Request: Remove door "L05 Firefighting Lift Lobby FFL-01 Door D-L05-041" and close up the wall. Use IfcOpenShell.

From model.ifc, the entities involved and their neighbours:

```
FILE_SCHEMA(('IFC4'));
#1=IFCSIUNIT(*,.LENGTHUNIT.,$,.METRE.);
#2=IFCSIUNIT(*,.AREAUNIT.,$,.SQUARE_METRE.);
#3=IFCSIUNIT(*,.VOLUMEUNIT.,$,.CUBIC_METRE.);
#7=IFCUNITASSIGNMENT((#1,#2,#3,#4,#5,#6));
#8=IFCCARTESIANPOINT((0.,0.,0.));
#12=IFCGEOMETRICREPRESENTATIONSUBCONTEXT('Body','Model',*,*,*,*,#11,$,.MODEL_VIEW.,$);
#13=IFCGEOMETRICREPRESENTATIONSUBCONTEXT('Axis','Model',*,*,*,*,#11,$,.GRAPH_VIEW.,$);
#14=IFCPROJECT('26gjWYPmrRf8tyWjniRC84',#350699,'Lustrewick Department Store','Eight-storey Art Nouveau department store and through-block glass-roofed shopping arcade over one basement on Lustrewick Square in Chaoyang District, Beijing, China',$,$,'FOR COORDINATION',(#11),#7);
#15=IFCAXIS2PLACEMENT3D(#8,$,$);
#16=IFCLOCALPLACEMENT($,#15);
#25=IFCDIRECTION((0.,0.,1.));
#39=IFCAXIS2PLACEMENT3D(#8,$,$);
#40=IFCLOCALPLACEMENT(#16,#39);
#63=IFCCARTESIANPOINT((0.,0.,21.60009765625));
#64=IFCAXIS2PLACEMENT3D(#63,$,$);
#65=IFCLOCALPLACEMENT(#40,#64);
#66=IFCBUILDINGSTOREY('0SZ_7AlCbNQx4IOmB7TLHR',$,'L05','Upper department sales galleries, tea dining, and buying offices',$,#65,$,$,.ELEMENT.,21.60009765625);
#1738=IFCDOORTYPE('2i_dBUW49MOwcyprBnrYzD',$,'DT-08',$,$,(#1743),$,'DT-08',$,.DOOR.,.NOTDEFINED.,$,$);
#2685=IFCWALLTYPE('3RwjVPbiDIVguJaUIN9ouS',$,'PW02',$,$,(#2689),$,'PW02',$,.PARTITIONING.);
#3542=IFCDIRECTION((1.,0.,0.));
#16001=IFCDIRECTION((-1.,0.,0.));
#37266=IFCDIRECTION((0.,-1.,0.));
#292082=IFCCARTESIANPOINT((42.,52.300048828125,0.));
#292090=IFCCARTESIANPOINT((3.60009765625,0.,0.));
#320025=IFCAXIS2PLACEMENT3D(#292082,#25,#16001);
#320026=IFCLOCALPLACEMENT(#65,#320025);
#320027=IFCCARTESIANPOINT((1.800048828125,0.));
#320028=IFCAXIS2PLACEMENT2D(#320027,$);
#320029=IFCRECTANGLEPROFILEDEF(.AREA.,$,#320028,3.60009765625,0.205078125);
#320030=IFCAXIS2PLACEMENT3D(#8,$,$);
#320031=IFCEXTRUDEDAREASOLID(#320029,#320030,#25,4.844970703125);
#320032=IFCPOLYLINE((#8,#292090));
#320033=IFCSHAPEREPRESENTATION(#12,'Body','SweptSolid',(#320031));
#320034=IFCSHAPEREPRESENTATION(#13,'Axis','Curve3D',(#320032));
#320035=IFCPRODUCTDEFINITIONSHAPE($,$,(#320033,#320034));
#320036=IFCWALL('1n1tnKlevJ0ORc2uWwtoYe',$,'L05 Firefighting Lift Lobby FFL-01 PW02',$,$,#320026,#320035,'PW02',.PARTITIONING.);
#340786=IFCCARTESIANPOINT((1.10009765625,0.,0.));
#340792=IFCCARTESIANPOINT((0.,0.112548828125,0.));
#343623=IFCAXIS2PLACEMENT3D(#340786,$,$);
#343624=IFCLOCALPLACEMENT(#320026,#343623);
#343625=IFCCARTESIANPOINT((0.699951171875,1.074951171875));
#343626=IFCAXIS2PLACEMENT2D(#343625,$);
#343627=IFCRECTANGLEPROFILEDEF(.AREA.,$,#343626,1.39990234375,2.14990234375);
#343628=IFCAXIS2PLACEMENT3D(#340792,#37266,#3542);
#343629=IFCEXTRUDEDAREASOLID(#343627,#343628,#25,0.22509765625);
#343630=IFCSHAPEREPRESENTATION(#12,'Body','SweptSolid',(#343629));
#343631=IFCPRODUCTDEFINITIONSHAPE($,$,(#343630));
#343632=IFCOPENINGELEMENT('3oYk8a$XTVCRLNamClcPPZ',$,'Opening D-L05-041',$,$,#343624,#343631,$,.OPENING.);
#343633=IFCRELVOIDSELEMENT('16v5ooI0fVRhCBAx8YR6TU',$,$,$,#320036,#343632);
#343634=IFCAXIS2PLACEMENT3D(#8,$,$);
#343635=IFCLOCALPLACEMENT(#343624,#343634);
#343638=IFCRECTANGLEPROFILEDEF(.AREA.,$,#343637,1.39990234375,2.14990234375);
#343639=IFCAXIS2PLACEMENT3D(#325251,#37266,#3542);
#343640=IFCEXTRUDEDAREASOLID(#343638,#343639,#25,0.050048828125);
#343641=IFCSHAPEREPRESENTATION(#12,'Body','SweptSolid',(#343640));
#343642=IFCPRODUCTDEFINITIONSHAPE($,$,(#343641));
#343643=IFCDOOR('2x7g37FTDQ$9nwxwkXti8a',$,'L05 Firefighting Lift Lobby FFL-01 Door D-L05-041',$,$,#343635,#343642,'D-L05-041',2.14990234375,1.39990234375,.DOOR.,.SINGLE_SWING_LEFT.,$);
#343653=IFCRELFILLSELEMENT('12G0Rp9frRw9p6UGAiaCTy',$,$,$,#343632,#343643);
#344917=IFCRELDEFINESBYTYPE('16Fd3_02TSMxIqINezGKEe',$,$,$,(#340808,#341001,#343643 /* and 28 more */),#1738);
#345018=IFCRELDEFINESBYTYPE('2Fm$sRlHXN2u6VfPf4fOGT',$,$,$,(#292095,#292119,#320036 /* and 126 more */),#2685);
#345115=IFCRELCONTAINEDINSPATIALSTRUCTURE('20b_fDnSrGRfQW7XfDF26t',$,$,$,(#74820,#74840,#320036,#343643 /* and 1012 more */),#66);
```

```python
import ifcopenshell
import ifcopenshell.api.feature
import ifcopenshell.api.root
import ifcopenshell.geom
import ifcopenshell.util.shape

model = ifcopenshell.open("model.ifc")
settings = ifcopenshell.geom.settings()


def volume(element):
    """Net volume in cubic metres, openings subtracted."""
    shape = ifcopenshell.geom.create_shape(settings, element)
    return ifcopenshell.util.shape.get_volume(shape.geometry)


door = model.by_id(343643)
opening = door.FillsVoids[0].RelatingOpeningElement
wall = opening.VoidsElements[0].RelatingBuildingElement
before = volume(wall)

ifcopenshell.api.root.remove_product(model, product=door)
ifcopenshell.api.feature.remove_feature(model, feature=opening)

after = volume(wall)

print(f"wall volume {before:.3f} -> {after:.3f} m3")

model.write("model-out.ifc")
```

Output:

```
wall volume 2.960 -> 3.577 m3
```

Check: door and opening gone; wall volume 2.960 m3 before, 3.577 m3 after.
